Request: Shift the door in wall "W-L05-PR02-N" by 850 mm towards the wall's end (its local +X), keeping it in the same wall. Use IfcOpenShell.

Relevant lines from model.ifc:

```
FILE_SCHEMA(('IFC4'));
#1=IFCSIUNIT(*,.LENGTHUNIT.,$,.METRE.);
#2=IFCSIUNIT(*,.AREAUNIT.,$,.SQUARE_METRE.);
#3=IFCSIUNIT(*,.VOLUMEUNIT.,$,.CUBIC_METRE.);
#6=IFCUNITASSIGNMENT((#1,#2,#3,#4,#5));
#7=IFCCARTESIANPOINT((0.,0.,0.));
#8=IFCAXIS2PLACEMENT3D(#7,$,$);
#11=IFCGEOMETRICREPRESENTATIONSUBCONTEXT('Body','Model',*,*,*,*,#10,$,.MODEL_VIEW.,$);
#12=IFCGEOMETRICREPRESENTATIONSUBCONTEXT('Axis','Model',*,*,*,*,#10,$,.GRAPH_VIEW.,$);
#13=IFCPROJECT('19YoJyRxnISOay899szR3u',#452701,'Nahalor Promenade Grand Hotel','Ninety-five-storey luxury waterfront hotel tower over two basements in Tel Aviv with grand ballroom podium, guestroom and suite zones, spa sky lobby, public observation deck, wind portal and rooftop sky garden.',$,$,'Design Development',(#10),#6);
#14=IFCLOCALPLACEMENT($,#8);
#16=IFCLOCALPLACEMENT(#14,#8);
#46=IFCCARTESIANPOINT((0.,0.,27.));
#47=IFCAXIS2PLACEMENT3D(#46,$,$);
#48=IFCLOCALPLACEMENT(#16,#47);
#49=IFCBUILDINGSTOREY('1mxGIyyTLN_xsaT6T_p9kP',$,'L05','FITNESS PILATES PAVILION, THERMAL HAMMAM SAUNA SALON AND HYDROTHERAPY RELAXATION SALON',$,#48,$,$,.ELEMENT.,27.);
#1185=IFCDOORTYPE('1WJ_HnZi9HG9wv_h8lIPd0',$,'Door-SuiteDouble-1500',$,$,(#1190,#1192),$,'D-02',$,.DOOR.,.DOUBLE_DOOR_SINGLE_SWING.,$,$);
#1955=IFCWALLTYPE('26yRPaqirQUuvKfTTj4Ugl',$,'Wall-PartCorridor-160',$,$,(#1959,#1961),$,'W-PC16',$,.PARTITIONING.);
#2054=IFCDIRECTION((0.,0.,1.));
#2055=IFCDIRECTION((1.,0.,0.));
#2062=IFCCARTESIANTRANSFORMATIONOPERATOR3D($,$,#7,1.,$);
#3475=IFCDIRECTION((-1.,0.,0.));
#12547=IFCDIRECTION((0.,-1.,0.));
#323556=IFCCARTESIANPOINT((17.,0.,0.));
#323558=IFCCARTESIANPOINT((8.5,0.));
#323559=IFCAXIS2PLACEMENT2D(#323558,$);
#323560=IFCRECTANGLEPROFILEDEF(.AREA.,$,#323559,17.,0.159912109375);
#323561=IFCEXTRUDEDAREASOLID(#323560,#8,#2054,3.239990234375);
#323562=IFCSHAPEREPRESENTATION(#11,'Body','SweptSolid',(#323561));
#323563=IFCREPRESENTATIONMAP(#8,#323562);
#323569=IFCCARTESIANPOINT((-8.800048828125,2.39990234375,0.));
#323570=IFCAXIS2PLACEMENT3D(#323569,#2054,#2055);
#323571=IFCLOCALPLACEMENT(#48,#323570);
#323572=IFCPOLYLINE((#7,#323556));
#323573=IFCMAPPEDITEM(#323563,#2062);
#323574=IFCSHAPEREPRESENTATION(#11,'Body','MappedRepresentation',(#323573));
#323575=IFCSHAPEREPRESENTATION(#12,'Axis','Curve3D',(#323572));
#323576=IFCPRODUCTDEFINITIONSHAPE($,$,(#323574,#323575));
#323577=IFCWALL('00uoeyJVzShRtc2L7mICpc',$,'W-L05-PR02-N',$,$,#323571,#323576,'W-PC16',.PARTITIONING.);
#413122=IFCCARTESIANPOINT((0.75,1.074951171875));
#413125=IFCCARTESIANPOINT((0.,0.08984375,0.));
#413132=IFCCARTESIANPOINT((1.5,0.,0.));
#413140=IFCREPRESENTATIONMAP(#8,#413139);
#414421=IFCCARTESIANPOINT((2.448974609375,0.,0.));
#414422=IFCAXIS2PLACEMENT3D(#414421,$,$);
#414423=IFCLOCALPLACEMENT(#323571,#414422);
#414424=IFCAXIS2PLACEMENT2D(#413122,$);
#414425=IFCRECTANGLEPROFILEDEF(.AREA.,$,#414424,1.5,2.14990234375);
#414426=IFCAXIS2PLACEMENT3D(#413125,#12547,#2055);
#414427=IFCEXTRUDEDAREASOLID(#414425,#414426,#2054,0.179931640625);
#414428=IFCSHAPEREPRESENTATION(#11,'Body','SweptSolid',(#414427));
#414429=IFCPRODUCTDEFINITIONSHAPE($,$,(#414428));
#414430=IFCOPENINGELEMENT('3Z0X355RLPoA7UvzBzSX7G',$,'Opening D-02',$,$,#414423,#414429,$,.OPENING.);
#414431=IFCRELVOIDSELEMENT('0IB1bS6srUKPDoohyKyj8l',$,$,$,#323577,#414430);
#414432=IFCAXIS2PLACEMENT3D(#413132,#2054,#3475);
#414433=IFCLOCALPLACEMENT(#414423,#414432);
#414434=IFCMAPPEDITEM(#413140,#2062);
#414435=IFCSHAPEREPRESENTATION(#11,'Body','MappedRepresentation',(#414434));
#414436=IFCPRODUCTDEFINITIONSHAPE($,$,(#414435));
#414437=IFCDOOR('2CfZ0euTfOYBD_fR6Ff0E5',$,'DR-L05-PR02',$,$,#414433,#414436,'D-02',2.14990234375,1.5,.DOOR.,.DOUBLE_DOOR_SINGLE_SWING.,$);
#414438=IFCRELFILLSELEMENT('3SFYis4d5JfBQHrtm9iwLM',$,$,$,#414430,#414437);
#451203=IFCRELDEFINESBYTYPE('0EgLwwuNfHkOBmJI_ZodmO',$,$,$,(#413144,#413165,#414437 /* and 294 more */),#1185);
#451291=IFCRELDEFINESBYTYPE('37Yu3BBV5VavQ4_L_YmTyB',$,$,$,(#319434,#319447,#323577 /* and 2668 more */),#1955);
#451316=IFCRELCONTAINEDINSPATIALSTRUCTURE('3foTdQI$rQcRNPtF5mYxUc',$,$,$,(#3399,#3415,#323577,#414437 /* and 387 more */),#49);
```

```python
import ifcopenshell
import ifcopenshell.api.geometry
import ifcopenshell.util.placement
import ifcopenshell.util.unit

model = ifcopenshell.open("model.ifc")
unit_scale = ifcopenshell.util.unit.calculate_unit_scale(model)

door = model.by_id(414437)
opening = door.FillsVoids[0].RelatingOpeningElement
wall = opening.VoidsElements[0].RelatingBuildingElement

wall_matrix = ifcopenshell.util.placement.get_local_placement(wall.ObjectPlacement)
shift = wall_matrix[:3, 0] * 0.85 / unit_scale
before = ifcopenshell.util.placement.get_local_placement(door.ObjectPlacement)[:3, 3].copy()

# The door is placed relative to its opening, so it follows when the opening moves.
matrix = ifcopenshell.util.placement.get_local_placement(opening.ObjectPlacement)
matrix[:3, 3] += shift
ifcopenshell.api.geometry.edit_object_placement(
    model, product=opening, matrix=matrix, is_si=False, should_transform_children=True
)

after = ifcopenshell.util.placement.get_local_placement(door.ObjectPlacement)[:3, 3]
print("door moved by", (after - before).round(3) + 0.0)

model.write("model_v2.ifc")
```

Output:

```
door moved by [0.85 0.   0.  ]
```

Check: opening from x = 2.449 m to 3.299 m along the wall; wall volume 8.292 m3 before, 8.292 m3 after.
